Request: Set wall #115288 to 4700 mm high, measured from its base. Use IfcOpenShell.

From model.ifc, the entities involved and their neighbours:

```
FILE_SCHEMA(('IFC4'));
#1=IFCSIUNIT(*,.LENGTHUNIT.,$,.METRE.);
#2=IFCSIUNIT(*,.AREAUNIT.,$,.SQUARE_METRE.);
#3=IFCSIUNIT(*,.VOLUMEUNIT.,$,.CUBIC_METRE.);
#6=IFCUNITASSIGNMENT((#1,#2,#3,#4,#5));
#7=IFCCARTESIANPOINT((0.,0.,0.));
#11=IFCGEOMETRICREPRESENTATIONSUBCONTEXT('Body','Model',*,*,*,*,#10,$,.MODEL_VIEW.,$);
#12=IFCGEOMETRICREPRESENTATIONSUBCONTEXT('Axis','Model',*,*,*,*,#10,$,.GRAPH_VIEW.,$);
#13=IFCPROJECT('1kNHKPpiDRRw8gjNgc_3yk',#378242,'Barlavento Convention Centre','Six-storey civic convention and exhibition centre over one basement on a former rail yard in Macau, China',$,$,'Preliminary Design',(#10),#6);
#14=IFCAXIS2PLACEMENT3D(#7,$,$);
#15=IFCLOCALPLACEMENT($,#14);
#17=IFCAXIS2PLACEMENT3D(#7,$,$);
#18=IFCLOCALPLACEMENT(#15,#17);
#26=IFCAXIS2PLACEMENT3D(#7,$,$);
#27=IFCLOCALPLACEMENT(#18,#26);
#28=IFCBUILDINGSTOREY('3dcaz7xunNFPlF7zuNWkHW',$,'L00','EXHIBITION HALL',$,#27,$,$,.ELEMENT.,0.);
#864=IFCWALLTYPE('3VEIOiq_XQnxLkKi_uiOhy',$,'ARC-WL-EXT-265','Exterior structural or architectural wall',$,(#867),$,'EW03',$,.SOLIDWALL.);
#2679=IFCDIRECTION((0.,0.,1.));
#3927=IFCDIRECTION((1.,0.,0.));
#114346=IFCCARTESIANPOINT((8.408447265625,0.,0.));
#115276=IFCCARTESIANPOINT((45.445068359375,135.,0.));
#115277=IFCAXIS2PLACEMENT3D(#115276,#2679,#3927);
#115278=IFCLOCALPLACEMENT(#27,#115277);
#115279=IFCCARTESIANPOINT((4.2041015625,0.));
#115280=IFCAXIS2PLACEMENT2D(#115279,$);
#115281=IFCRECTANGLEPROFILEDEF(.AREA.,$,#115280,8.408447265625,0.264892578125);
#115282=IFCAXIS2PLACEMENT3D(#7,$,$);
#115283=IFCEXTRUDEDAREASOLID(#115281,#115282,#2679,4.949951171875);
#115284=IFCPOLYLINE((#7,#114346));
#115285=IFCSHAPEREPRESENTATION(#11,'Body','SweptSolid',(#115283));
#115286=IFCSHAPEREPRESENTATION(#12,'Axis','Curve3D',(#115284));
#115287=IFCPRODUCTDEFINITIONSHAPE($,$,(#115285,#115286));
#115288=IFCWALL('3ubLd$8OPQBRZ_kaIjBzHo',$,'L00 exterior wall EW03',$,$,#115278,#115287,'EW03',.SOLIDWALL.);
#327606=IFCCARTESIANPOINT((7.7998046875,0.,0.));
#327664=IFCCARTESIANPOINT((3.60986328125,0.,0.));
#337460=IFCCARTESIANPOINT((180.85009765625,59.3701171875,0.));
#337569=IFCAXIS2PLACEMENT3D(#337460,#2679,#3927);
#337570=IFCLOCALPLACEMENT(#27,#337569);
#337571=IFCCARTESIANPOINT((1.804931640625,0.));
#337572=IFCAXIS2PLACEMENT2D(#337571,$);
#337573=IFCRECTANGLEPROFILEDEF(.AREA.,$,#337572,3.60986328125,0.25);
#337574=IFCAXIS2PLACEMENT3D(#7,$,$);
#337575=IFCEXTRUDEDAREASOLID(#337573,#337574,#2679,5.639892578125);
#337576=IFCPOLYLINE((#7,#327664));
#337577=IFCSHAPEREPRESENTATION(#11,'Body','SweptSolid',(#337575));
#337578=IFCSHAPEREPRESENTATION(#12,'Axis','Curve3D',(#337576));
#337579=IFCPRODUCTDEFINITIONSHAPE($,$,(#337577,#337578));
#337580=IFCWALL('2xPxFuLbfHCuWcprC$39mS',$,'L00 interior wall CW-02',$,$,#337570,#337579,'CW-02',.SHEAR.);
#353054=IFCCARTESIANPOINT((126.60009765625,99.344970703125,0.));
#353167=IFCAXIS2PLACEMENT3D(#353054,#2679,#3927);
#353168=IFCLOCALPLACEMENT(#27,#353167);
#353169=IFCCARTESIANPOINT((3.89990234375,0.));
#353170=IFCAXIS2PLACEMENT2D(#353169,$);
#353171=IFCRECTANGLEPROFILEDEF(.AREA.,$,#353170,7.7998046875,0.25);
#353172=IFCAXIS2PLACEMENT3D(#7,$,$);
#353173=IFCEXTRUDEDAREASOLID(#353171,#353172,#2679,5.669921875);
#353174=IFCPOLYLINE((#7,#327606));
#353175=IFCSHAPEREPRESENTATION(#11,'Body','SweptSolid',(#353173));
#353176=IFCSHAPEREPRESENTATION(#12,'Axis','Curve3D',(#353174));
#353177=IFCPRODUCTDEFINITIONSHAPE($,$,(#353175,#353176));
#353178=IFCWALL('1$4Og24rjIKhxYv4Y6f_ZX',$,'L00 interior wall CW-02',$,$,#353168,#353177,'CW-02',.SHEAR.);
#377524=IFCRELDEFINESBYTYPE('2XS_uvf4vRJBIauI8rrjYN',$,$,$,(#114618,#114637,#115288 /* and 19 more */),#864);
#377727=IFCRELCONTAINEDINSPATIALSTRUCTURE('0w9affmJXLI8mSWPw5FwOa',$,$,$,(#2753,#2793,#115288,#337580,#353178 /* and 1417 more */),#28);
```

```python
import ifcopenshell
import ifcopenshell.geom
import ifcopenshell.util.representation
import ifcopenshell.util.shape

model = ifcopenshell.open("model.ifc")
settings = ifcopenshell.geom.settings()


def volume(element):
    """Net volume in cubic metres, openings subtracted."""
    shape = ifcopenshell.geom.create_shape(settings, element)
    return ifcopenshell.util.shape.get_volume(shape.geometry)


wall = model.by_id(115288)
before = volume(wall)

body = ifcopenshell.util.representation.get_representation(wall, "Model", "Body")
solid = body.Items[0]
old_height = solid.Depth
solid.Depth = 4.7
after = volume(wall)

print(f"height {old_height:g} -> {solid.Depth:g}, volume {before:.3f} -> {after:.3f} m3")

model.write("model_updated.ifc")
```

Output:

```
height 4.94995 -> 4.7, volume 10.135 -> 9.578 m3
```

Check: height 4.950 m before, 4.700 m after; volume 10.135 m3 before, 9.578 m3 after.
